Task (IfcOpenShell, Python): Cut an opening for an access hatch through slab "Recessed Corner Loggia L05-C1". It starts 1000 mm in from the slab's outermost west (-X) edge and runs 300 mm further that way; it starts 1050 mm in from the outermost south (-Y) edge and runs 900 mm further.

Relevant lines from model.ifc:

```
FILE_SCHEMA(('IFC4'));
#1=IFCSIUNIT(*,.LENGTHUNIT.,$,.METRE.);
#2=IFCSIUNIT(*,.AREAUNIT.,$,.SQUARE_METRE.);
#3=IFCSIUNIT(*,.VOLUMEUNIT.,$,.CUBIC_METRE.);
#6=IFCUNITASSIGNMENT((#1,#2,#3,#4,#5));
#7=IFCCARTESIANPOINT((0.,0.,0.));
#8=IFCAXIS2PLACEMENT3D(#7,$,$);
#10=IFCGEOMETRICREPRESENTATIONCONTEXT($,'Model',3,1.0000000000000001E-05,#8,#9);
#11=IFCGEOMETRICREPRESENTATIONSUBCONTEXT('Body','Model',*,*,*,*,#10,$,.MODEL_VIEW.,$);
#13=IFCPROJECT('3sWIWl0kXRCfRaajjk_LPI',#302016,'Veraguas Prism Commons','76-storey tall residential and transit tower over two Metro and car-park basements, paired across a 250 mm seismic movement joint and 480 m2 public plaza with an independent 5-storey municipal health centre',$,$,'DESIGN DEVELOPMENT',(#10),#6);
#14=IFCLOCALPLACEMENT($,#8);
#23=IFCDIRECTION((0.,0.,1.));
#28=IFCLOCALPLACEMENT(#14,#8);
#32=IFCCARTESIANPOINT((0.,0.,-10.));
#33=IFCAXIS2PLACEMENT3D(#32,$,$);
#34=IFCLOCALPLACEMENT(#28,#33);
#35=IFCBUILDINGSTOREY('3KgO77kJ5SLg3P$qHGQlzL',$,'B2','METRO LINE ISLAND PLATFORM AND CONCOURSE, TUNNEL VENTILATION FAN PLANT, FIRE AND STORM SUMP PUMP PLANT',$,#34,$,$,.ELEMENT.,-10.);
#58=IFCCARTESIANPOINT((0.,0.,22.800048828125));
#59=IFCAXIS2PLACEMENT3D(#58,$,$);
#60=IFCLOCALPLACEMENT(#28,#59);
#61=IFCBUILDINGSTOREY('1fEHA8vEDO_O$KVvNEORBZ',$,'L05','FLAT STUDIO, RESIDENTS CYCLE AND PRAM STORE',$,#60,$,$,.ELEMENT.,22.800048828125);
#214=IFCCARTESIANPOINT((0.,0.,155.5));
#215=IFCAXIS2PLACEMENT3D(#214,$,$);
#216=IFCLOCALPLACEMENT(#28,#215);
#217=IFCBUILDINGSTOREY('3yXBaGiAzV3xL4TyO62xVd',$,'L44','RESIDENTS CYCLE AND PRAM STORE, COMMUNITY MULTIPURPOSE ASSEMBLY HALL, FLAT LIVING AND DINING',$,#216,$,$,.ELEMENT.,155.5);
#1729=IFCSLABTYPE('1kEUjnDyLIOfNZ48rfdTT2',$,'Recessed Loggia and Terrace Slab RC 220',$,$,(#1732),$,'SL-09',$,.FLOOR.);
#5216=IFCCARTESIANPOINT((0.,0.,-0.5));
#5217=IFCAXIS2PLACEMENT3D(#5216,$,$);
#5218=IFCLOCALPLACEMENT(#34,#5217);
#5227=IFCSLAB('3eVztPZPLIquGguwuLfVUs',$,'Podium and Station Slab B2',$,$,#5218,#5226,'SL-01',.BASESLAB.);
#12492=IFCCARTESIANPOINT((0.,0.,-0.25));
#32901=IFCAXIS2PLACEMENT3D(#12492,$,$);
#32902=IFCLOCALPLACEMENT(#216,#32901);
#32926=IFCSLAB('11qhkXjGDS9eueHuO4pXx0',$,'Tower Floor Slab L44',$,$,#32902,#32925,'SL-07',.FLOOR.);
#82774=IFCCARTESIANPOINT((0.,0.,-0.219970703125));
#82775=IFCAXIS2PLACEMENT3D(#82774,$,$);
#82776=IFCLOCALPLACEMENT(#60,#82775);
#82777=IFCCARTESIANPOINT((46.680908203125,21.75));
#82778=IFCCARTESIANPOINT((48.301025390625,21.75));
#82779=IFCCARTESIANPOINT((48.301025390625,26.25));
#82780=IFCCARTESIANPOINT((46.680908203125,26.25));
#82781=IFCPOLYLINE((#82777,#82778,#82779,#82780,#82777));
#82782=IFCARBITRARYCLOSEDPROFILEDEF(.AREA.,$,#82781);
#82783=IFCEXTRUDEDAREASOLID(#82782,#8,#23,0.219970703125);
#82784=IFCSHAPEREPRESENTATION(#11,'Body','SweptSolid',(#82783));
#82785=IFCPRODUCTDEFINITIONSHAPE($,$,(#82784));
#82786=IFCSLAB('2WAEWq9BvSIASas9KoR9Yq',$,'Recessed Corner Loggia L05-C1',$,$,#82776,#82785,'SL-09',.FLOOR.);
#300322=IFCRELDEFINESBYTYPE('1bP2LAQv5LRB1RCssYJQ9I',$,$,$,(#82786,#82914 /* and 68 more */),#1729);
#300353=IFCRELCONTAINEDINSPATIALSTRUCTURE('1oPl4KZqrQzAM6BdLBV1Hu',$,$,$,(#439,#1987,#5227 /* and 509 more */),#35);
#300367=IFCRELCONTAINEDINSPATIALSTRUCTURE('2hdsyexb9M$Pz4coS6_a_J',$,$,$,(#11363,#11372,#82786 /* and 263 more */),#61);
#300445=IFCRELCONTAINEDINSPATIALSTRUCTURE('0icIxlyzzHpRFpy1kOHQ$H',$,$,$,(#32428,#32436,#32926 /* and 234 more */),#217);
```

```python
import numpy as np
import ifcopenshell
import ifcopenshell.api.feature
import ifcopenshell.api.geometry
import ifcopenshell.api.root
import ifcopenshell.geom
import ifcopenshell.util.placement
import ifcopenshell.util.representation
import ifcopenshell.util.shape
import ifcopenshell.util.unit

model = ifcopenshell.open("model.ifc")
unit_scale = ifcopenshell.util.unit.calculate_unit_scale(model)
settings = ifcopenshell.geom.settings()


def volume(element):
    """Net volume in cubic metres, openings subtracted."""
    shape = ifcopenshell.geom.create_shape(settings, element)
    return ifcopenshell.util.shape.get_volume(shape.geometry)


slab = model.by_guid("2WAEWq9BvSIASas9KoR9Yq")
before = volume(slab)

# Extent in the slab's own axes, in metres. The edges named are its -X and -Y sides.
slab_shape = ifcopenshell.geom.create_shape(settings, slab)
vertices = ifcopenshell.util.shape.get_vertices(slab_shape.geometry)
x_min, y_min, bottom = vertices.min(axis=0)
top = vertices[:, 2].max()

opening = ifcopenshell.api.root.create_entity(model, ifc_class="IfcOpeningElement", name="Access hatch opening", predefined_type="OPENING")
context = ifcopenshell.util.representation.get_context(model, "Model", "Body", "MODEL_VIEW")
width, depth = 0.3, 0.9
outline = [(0.0, 0.0), (width, 0.0), (width, depth), (0.0, depth), (0.0, 0.0)]
# Overshoot both faces by 50 mm so the cut is clean.
shape = ifcopenshell.api.geometry.add_slab_representation(
    model, context=context, depth=top - bottom + 0.1, polyline=outline
)
ifcopenshell.api.geometry.assign_representation(model, product=opening, representation=shape)

matrix = ifcopenshell.util.placement.get_local_placement(slab.ObjectPlacement)
matrix[:, 3] = matrix @ np.append(np.array([x_min + 1, y_min + 1.05, bottom - 0.05]) / unit_scale, 1.0)
ifcopenshell.api.geometry.edit_object_placement(model, product=opening, matrix=matrix, is_si=False)
ifcopenshell.api.feature.add_feature(model, feature=opening, element=slab)

after = volume(slab)

print(f"slab volume {before:.3f} -> {after:.3f} m3")

model.write("model-out.ifc")
```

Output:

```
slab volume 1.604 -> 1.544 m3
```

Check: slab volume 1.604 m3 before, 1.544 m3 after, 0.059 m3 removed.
